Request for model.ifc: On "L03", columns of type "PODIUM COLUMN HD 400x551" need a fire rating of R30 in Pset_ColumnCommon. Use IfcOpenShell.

First a look at what the model holds.

```python
import ifcopenshell
import ifcopenshell.util.element

model = ifcopenshell.open("model.ifc")
print(model.schema)
storey = next(s for s in model.by_type("IfcBuildingStorey") if s.Name == "L03")
columns = [e for e in ifcopenshell.util.element.get_decomposition(storey) if e.is_a("IfcColumn")]
seen = {}
for e in columns:
    element_type = ifcopenshell.util.element.get_type(e)
    key = (element_type.Name if element_type != e and element_type else None, ifcopenshell.util.element.get_pset(e, "Pset_ColumnCommon", "FireRating"))
    seen[key] = seen.get(key, 0) + 1
for (name, value), count in sorted(seen.items(), key=str):
    print(count, "x", name, "|", value)
```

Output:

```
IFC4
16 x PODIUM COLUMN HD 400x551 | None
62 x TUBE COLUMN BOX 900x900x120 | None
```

```python
import ifcopenshell
import ifcopenshell.api.pset
import ifcopenshell.util.element

model = ifcopenshell.open("model.ifc")

storey = next(s for s in model.by_type("IfcBuildingStorey") if s.Name == "L03")
columns = [e for e in ifcopenshell.util.element.get_decomposition(storey) if e.is_a("IfcColumn")]

count = 0
for e in columns:
    element_type = ifcopenshell.util.element.get_type(e)
    if element_type in (None, e) or element_type.Name != "PODIUM COLUMN HD 400x551":
        continue
    found = ifcopenshell.util.element.get_pset(e, "Pset_ColumnCommon", should_inherit=False)
    if found:
        pset = model.by_id(found["id"])
        if len(ifcopenshell.util.element.get_elements_by_pset(pset)) > 1:
            pset = ifcopenshell.api.pset.unshare_pset(model, products=[e], pset=pset)[0]
    else:
        pset = ifcopenshell.api.pset.add_pset(model, product=e, name="Pset_ColumnCommon")
    ifcopenshell.api.pset.edit_pset(model, pset=pset, properties={"FireRating": "R30"})
    count += 1

print(count, "columns updated")

model.write("model_rev.ifc")
```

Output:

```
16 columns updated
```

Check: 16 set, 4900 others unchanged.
